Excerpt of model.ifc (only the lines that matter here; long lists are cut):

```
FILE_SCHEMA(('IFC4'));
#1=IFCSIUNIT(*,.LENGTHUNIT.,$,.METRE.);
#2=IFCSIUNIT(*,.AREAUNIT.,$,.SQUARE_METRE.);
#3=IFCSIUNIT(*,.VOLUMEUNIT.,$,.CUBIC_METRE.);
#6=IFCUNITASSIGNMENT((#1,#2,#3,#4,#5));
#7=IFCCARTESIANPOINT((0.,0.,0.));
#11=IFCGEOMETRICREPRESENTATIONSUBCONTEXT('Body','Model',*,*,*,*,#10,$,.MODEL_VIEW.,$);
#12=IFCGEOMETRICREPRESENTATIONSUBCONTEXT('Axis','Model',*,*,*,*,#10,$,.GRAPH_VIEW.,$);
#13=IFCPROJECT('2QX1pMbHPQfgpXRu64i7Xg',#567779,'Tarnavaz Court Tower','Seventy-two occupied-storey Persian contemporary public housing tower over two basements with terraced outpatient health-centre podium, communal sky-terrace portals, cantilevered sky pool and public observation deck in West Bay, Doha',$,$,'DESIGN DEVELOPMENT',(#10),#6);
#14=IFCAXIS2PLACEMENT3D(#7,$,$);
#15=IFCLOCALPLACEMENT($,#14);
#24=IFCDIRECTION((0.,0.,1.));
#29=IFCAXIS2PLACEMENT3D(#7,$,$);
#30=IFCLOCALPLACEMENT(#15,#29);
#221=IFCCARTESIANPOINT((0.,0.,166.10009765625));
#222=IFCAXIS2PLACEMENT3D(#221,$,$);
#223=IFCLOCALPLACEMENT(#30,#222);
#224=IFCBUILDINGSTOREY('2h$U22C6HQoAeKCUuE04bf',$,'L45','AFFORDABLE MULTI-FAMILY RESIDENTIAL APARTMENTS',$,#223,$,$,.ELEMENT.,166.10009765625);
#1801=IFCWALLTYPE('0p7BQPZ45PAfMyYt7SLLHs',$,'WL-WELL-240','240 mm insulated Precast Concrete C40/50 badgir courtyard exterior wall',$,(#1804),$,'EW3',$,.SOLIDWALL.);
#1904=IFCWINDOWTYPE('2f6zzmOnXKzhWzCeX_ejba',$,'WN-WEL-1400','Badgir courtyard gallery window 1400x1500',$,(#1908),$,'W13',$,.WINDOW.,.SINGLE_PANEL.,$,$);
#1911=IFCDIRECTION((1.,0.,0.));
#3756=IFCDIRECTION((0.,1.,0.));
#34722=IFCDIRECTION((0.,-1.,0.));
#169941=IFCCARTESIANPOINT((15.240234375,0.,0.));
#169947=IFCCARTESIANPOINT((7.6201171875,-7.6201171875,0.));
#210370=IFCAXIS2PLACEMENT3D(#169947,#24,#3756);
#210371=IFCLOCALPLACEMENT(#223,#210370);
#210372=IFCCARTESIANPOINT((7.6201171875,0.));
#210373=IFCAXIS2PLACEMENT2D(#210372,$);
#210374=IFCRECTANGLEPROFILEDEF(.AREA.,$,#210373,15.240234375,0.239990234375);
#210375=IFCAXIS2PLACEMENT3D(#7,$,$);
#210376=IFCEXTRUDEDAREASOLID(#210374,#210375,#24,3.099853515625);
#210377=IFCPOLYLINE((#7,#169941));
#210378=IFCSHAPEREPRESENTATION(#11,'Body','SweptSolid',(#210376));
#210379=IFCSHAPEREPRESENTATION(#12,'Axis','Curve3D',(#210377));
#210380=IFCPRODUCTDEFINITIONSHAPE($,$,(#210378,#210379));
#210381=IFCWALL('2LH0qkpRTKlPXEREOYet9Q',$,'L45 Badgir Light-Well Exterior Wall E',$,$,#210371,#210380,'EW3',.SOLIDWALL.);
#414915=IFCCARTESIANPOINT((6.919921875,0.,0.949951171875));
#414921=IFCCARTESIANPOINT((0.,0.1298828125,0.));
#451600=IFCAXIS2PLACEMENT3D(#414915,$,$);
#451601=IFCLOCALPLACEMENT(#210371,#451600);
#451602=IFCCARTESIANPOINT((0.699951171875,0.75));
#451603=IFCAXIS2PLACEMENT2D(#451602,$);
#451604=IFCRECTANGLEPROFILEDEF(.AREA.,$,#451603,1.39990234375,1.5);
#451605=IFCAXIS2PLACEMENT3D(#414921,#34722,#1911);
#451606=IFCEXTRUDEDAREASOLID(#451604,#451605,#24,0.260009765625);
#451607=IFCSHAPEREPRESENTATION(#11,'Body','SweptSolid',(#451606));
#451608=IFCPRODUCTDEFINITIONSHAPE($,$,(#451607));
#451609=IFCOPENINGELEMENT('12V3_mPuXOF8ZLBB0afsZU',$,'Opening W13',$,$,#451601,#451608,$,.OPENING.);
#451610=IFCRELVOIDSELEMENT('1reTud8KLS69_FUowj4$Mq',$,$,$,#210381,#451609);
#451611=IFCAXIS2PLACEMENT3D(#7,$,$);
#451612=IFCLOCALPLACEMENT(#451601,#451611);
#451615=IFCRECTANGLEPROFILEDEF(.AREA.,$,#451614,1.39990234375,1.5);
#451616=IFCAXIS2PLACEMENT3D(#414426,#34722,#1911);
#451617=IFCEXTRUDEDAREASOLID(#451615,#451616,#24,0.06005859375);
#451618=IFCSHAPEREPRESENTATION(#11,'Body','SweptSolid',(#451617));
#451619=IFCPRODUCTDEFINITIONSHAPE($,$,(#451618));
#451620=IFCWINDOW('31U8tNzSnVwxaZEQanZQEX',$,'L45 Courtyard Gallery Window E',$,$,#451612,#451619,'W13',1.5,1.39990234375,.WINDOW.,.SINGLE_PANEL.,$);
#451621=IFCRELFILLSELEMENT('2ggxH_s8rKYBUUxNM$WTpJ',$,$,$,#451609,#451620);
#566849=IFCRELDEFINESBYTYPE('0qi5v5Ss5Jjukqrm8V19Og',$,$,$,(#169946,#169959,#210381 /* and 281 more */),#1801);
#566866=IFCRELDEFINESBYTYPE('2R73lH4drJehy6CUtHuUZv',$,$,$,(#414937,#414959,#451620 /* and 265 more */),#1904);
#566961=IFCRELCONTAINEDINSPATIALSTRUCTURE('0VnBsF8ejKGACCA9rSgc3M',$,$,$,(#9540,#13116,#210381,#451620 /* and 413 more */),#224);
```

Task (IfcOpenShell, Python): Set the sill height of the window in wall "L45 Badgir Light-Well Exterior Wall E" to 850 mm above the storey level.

```python
import numpy as np
import ifcopenshell
import ifcopenshell.api.geometry
import ifcopenshell.geom
import ifcopenshell.util.element
import ifcopenshell.util.placement
import ifcopenshell.util.shape
import ifcopenshell.util.unit

model = ifcopenshell.open("model.ifc")
unit_scale = ifcopenshell.util.unit.calculate_unit_scale(model)

window = model.by_guid("31U8tNzSnVwxaZEQanZQEX")
opening = window.FillsVoids[0].RelatingOpeningElement
storey = ifcopenshell.util.element.get_container(window, ifc_class="IfcBuildingStorey")
level = ifcopenshell.util.placement.get_local_placement(storey.ObjectPlacement)[2, 3]

# The opening's origin need not be at the sill, so measure its lowest point.
shape = ifcopenshell.geom.create_shape(ifcopenshell.geom.settings(), opening)
bottom = ifcopenshell.util.shape.get_shape_bottom_elevation(shape, shape.geometry) / unit_scale
dz = level + 0.85 - bottom

shift = np.array([0.0, 0.0, dz])
# The window is placed relative to its opening, so it follows when the opening moves.
matrix = ifcopenshell.util.placement.get_local_placement(opening.ObjectPlacement)
matrix[:3, 3] += shift
ifcopenshell.api.geometry.edit_object_placement(
    model, product=opening, matrix=matrix, is_si=False, should_transform_children=True
)

print(f"moved by {dz * unit_scale:+.3f} m")

model.write("model-out.ifc")
```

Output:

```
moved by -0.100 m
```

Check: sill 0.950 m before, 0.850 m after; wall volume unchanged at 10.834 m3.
